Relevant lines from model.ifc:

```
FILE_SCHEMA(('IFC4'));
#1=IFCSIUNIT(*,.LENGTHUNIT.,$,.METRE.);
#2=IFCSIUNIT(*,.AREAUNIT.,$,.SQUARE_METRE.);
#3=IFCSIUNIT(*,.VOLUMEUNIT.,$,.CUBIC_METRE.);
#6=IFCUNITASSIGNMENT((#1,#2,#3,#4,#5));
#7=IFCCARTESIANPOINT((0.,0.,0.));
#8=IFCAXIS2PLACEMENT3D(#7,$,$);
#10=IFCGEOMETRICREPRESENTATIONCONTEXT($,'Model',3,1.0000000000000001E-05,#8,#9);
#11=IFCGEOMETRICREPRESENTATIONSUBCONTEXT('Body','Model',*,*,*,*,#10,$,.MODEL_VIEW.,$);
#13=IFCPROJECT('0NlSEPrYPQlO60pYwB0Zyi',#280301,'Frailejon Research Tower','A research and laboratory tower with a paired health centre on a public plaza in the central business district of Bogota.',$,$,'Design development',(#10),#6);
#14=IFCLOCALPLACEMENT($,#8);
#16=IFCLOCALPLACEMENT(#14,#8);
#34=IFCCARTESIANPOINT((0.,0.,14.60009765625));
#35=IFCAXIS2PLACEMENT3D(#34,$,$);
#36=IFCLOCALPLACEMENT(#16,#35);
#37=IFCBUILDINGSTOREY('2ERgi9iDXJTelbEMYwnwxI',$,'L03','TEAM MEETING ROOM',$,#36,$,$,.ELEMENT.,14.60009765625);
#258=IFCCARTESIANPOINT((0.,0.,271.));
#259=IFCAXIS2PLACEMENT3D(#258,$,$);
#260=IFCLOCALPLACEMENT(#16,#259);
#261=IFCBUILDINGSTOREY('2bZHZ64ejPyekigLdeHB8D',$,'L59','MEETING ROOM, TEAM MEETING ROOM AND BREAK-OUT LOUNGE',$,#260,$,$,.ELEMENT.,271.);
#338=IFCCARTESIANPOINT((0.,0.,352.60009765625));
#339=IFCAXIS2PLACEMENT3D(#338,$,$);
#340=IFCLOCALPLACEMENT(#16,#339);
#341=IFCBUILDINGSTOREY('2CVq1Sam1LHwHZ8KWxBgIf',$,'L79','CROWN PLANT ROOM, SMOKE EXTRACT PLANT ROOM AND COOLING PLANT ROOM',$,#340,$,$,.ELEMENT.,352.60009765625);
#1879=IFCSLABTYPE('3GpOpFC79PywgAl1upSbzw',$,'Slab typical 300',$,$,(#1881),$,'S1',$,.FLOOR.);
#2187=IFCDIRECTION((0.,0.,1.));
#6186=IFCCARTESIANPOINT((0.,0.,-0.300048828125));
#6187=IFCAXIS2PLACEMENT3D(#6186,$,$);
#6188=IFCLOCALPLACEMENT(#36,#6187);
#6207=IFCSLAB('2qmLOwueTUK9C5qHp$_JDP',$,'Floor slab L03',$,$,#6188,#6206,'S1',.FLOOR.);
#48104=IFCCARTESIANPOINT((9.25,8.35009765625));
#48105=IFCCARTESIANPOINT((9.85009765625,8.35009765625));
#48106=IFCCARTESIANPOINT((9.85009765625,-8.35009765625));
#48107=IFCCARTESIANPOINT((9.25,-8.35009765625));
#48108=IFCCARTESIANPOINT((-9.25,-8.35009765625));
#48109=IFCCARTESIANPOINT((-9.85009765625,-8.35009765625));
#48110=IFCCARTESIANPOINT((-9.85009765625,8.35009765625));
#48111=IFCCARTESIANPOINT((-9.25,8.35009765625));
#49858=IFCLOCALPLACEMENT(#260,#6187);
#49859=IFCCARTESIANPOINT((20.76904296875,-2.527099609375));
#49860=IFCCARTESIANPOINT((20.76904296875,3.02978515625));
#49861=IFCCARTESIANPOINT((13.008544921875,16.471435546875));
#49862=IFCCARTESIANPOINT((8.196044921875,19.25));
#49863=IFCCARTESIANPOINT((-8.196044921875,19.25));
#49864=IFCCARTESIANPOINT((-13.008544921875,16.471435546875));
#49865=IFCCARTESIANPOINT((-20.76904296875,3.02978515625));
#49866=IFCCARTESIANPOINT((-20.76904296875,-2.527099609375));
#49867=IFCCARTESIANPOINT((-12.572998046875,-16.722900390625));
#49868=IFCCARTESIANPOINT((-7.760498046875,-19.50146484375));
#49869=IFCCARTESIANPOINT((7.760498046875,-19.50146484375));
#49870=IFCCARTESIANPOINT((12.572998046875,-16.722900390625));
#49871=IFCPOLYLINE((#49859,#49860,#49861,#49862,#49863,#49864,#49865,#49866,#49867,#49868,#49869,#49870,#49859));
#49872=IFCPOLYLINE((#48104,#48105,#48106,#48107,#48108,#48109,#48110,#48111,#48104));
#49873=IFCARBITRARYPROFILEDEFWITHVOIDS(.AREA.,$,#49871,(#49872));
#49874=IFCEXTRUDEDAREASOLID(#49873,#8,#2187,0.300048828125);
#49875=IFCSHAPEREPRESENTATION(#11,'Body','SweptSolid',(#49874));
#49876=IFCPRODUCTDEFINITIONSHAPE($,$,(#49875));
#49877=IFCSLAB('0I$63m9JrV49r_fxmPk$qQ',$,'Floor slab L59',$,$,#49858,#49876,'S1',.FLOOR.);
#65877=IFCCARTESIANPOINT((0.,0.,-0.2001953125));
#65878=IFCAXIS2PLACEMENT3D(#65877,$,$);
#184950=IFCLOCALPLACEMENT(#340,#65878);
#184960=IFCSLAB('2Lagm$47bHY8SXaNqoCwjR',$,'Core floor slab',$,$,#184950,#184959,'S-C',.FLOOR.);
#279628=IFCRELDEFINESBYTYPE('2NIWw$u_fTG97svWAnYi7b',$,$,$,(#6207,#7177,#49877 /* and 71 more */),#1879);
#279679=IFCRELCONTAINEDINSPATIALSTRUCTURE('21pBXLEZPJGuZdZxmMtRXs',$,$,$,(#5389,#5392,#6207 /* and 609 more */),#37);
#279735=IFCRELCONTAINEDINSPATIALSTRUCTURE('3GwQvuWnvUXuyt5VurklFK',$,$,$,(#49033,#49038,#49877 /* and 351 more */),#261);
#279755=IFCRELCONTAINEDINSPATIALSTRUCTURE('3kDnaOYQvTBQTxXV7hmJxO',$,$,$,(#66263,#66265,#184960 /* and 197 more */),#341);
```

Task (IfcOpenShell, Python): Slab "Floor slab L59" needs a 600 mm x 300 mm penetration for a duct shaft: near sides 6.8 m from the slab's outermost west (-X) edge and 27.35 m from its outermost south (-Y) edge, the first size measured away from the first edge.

```python
import numpy as np
import ifcopenshell
import ifcopenshell.api.feature
import ifcopenshell.api.geometry
import ifcopenshell.api.root
import ifcopenshell.geom
import ifcopenshell.util.placement
import ifcopenshell.util.representation
import ifcopenshell.util.shape
import ifcopenshell.util.unit

model = ifcopenshell.open("model.ifc")
unit_scale = ifcopenshell.util.unit.calculate_unit_scale(model)
settings = ifcopenshell.geom.settings()


def volume(element):
    """Net volume in cubic metres, openings subtracted."""
    shape = ifcopenshell.geom.create_shape(settings, element)
    return ifcopenshell.util.shape.get_volume(shape.geometry)


slab = model.by_guid("0I$63m9JrV49r_fxmPk$qQ")
before = volume(slab)

# Extent in the slab's own axes, in metres. The edges named are its -X and -Y sides.
slab_shape = ifcopenshell.geom.create_shape(settings, slab)
vertices = ifcopenshell.util.shape.get_vertices(slab_shape.geometry)
x_min, y_min, bottom = vertices.min(axis=0)
top = vertices[:, 2].max()

opening = ifcopenshell.api.root.create_entity(model, ifc_class="IfcOpeningElement", name="Duct shaft opening", predefined_type="OPENING")
context = ifcopenshell.util.representation.get_context(model, "Model", "Body", "MODEL_VIEW")
width, depth = 0.6, 0.3
outline = [(0.0, 0.0), (width, 0.0), (width, depth), (0.0, depth), (0.0, 0.0)]
# Overshoot both faces by 50 mm so the cut is clean.
shape = ifcopenshell.api.geometry.add_slab_representation(
    model, context=context, depth=top - bottom + 0.1, polyline=outline
)
ifcopenshell.api.geometry.assign_representation(model, product=opening, representation=shape)

matrix = ifcopenshell.util.placement.get_local_placement(slab.ObjectPlacement)
matrix[:, 3] = matrix @ np.append(np.array([x_min + 6.8, y_min + 27.35, bottom - 0.05]) / unit_scale, 1.0)
ifcopenshell.api.geometry.edit_object_placement(model, product=opening, matrix=matrix, is_si=False)
ifcopenshell.api.feature.add_feature(model, feature=opening, element=slab)

after = volume(slab)

print(f"slab volume {before:.3f} -> {after:.3f} m3")

model.write("model_v2.ifc")
```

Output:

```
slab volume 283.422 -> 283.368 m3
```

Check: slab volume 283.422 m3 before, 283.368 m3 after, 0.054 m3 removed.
